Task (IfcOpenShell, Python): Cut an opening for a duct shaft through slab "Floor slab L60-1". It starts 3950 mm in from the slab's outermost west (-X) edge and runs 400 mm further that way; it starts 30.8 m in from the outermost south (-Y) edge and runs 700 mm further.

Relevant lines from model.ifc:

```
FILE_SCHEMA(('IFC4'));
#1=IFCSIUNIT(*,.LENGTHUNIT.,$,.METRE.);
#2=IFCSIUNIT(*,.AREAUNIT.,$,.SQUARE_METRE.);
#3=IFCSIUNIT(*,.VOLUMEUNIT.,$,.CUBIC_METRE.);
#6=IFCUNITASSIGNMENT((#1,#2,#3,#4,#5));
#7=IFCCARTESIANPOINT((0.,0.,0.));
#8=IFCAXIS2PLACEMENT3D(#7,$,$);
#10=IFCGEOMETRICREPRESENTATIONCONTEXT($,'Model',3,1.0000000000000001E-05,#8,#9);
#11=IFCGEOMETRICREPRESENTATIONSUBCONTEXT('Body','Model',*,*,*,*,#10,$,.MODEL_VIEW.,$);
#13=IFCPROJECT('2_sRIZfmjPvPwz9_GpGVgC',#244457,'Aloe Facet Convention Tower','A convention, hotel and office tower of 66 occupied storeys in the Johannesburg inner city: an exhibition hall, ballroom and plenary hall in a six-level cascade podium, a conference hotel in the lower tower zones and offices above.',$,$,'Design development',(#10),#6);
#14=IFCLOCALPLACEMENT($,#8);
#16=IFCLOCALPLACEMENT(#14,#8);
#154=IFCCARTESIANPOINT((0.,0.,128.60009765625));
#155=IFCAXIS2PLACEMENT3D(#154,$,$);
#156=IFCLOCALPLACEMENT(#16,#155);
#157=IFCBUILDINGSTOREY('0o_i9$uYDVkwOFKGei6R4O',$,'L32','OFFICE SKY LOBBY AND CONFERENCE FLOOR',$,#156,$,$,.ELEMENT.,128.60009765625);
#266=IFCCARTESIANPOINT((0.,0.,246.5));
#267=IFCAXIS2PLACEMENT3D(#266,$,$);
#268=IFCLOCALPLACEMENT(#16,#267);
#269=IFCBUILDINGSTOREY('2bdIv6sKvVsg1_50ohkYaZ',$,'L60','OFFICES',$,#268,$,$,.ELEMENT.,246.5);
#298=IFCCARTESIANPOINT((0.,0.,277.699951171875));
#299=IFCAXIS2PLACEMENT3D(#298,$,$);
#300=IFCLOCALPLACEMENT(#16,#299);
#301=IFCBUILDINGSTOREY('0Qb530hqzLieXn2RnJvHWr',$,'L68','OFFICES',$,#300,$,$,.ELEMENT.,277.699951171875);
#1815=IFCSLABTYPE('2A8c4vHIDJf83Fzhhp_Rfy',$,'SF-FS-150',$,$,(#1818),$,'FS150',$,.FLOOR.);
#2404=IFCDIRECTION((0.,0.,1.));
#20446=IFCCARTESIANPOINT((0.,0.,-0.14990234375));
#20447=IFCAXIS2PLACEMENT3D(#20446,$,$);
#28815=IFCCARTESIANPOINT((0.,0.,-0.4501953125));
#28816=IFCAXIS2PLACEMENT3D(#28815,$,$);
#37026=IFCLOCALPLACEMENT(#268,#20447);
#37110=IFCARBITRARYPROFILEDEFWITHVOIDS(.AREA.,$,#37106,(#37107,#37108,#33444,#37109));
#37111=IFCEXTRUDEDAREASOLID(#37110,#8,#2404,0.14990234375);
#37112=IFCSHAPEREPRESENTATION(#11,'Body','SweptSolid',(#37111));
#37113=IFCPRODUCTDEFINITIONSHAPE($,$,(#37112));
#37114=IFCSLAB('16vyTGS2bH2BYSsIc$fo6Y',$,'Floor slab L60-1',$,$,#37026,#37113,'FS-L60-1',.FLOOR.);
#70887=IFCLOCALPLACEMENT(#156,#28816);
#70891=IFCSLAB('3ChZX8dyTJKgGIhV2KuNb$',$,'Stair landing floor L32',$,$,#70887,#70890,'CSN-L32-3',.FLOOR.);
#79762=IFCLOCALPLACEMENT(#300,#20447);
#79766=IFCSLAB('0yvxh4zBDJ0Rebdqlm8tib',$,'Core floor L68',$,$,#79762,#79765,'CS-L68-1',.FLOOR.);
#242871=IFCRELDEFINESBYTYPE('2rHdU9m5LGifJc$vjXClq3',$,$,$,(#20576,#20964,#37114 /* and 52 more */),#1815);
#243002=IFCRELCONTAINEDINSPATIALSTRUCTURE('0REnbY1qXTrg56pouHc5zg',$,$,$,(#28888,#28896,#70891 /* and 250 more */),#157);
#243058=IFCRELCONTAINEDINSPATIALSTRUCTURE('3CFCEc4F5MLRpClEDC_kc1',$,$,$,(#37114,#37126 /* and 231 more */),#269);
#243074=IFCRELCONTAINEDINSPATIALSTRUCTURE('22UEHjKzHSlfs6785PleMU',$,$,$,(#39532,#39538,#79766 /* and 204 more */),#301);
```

```python
import numpy as np
import ifcopenshell
import ifcopenshell.api.feature
import ifcopenshell.api.geometry
import ifcopenshell.api.root
import ifcopenshell.geom
import ifcopenshell.util.placement
import ifcopenshell.util.representation
import ifcopenshell.util.shape
import ifcopenshell.util.unit

model = ifcopenshell.open("model.ifc")
unit_scale = ifcopenshell.util.unit.calculate_unit_scale(model)
settings = ifcopenshell.geom.settings()


def volume(element):
    """Net volume in cubic metres, openings subtracted."""
    shape = ifcopenshell.geom.create_shape(settings, element)
    return ifcopenshell.util.shape.get_volume(shape.geometry)


slab = model.by_guid("16vyTGS2bH2BYSsIc$fo6Y")
before = volume(slab)

# Extent in the slab's own axes, in metres. The edges named are its -X and -Y sides.
slab_shape = ifcopenshell.geom.create_shape(settings, slab)
vertices = ifcopenshell.util.shape.get_vertices(slab_shape.geometry)
x_min, y_min, bottom = vertices.min(axis=0)
top = vertices[:, 2].max()

opening = ifcopenshell.api.root.create_entity(model, ifc_class="IfcOpeningElement", name="Duct shaft opening", predefined_type="OPENING")
context = ifcopenshell.util.representation.get_context(model, "Model", "Body", "MODEL_VIEW")
width, depth = 0.4, 0.7
outline = [(0.0, 0.0), (width, 0.0), (width, depth), (0.0, depth), (0.0, 0.0)]
# Overshoot both faces by 50 mm so the cut is clean.
shape = ifcopenshell.api.geometry.add_slab_representation(
    model, context=context, depth=top - bottom + 0.1, polyline=outline
)
ifcopenshell.api.geometry.assign_representation(model, product=opening, representation=shape)

matrix = ifcopenshell.util.placement.get_local_placement(slab.ObjectPlacement)
matrix[:, 3] = matrix @ np.append(np.array([x_min + 3.95, y_min + 30.8, bottom - 0.05]) / unit_scale, 1.0)
ifcopenshell.api.geometry.edit_object_placement(model, product=opening, matrix=matrix, is_si=False)
ifcopenshell.api.feature.add_feature(model, feature=opening, element=slab)

after = volume(slab)

print(f"slab volume {before:.3f} -> {after:.3f} m3")

model.write("model_rev.ifc")
```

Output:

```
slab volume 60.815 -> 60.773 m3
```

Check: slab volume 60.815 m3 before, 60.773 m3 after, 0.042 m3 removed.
